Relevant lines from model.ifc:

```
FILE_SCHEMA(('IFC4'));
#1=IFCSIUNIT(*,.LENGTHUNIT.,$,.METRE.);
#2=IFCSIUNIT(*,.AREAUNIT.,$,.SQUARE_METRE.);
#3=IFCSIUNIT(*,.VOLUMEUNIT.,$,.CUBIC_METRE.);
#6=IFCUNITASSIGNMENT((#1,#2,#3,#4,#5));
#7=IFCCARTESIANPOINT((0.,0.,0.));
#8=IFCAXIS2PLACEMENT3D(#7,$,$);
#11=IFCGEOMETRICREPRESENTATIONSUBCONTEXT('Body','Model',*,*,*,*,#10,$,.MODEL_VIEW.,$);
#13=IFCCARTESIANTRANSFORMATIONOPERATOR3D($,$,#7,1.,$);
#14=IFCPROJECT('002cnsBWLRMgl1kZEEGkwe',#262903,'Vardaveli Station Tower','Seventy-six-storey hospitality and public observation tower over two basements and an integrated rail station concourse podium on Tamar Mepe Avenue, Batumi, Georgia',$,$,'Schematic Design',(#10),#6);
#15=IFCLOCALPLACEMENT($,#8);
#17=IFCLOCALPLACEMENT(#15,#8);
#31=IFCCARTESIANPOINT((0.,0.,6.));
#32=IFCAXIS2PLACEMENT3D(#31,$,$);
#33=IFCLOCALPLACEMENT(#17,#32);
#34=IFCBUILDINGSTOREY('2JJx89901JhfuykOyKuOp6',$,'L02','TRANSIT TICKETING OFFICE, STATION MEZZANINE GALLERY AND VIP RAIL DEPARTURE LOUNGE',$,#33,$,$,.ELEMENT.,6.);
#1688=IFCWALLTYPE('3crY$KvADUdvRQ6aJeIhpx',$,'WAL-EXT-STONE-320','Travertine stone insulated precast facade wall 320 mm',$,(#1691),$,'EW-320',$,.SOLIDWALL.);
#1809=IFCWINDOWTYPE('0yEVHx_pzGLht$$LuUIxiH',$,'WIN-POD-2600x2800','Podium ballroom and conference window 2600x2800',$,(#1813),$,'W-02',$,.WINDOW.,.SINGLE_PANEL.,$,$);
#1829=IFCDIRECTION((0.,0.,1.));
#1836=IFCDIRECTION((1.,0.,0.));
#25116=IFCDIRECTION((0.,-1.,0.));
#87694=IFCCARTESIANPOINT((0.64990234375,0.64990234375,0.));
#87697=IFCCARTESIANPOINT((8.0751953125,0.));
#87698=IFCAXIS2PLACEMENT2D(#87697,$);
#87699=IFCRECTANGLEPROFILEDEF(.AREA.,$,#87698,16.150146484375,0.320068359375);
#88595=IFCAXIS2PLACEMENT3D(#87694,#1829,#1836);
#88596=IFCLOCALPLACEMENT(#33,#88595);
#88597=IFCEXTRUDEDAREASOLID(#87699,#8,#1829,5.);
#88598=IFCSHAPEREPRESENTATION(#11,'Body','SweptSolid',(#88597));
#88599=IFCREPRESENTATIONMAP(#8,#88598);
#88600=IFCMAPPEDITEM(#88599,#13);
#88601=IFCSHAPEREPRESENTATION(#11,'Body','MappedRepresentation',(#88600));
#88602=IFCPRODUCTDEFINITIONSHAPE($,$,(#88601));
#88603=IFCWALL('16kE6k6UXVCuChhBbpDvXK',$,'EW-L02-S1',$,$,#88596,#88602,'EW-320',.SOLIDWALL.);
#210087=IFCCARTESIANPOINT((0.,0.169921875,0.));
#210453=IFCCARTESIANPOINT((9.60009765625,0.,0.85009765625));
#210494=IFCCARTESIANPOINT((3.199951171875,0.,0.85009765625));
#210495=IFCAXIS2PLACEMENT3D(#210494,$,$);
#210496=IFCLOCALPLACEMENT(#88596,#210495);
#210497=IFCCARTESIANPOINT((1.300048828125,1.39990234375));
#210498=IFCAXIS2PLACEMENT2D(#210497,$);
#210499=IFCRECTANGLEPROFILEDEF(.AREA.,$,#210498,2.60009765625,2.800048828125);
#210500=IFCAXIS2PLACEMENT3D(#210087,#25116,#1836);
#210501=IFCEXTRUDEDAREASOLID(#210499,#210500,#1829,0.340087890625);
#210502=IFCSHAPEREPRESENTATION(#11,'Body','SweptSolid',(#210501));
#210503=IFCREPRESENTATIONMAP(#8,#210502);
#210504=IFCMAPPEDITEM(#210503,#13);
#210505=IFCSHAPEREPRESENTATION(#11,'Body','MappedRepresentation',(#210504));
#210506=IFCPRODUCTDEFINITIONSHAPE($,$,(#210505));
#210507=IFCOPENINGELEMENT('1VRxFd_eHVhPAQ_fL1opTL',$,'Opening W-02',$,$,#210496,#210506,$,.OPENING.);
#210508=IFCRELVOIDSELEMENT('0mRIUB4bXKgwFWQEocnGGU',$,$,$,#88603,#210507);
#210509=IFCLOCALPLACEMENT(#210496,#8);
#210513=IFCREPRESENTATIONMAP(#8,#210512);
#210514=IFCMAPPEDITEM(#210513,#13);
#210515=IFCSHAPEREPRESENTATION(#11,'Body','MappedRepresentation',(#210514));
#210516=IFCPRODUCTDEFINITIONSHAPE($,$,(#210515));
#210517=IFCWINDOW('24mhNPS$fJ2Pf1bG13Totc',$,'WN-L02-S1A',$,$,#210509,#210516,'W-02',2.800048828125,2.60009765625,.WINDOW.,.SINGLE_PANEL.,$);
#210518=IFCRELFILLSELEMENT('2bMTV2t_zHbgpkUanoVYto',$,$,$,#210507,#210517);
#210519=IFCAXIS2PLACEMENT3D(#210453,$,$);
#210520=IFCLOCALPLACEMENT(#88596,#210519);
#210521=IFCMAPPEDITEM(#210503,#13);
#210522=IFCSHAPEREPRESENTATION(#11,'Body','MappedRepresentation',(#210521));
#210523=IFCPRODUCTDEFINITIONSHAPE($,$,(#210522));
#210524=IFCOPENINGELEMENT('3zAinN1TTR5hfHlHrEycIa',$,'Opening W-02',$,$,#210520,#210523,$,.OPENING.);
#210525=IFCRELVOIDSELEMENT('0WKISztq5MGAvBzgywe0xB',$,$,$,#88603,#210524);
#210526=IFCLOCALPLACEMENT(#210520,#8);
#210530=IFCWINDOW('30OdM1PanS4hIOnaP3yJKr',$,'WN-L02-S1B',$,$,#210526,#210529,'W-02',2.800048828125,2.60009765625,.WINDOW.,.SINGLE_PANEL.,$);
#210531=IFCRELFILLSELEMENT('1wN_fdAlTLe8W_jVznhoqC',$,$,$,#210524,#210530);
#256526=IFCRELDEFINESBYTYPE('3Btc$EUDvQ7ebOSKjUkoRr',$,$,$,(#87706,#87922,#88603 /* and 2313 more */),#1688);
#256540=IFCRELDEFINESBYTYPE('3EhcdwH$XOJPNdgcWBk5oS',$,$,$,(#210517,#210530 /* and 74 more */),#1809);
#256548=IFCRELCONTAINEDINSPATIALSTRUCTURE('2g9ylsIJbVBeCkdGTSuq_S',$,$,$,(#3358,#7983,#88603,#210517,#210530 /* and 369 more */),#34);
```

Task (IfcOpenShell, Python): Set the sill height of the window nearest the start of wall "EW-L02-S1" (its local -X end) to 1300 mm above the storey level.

```python
import numpy as np
import ifcopenshell
import ifcopenshell.api.geometry
import ifcopenshell.geom
import ifcopenshell.util.element
import ifcopenshell.util.placement
import ifcopenshell.util.shape
import ifcopenshell.util.unit

model = ifcopenshell.open("model.ifc")
unit_scale = ifcopenshell.util.unit.calculate_unit_scale(model)

window = model.by_guid("24mhNPS$fJ2Pf1bG13Totc")
opening = window.FillsVoids[0].RelatingOpeningElement
storey = ifcopenshell.util.element.get_container(window, ifc_class="IfcBuildingStorey")
level = ifcopenshell.util.placement.get_local_placement(storey.ObjectPlacement)[2, 3]

# The opening's origin need not be at the sill, so measure its lowest point.
shape = ifcopenshell.geom.create_shape(ifcopenshell.geom.settings(), opening)
bottom = ifcopenshell.util.shape.get_shape_bottom_elevation(shape, shape.geometry) / unit_scale
dz = level + 1.3 / unit_scale - bottom

shift = np.array([0.0, 0.0, dz])
# The window is placed relative to its opening, so it follows when the opening moves.
matrix = ifcopenshell.util.placement.get_local_placement(opening.ObjectPlacement)
matrix[:3, 3] += shift
ifcopenshell.api.geometry.edit_object_placement(
    model, product=opening, matrix=matrix, is_si=False, should_transform_children=True
)

print(f"moved by {dz * unit_scale:+.3f} m")

model.write("model_v2.ifc")
```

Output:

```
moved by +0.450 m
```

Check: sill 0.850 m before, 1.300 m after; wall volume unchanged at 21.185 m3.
